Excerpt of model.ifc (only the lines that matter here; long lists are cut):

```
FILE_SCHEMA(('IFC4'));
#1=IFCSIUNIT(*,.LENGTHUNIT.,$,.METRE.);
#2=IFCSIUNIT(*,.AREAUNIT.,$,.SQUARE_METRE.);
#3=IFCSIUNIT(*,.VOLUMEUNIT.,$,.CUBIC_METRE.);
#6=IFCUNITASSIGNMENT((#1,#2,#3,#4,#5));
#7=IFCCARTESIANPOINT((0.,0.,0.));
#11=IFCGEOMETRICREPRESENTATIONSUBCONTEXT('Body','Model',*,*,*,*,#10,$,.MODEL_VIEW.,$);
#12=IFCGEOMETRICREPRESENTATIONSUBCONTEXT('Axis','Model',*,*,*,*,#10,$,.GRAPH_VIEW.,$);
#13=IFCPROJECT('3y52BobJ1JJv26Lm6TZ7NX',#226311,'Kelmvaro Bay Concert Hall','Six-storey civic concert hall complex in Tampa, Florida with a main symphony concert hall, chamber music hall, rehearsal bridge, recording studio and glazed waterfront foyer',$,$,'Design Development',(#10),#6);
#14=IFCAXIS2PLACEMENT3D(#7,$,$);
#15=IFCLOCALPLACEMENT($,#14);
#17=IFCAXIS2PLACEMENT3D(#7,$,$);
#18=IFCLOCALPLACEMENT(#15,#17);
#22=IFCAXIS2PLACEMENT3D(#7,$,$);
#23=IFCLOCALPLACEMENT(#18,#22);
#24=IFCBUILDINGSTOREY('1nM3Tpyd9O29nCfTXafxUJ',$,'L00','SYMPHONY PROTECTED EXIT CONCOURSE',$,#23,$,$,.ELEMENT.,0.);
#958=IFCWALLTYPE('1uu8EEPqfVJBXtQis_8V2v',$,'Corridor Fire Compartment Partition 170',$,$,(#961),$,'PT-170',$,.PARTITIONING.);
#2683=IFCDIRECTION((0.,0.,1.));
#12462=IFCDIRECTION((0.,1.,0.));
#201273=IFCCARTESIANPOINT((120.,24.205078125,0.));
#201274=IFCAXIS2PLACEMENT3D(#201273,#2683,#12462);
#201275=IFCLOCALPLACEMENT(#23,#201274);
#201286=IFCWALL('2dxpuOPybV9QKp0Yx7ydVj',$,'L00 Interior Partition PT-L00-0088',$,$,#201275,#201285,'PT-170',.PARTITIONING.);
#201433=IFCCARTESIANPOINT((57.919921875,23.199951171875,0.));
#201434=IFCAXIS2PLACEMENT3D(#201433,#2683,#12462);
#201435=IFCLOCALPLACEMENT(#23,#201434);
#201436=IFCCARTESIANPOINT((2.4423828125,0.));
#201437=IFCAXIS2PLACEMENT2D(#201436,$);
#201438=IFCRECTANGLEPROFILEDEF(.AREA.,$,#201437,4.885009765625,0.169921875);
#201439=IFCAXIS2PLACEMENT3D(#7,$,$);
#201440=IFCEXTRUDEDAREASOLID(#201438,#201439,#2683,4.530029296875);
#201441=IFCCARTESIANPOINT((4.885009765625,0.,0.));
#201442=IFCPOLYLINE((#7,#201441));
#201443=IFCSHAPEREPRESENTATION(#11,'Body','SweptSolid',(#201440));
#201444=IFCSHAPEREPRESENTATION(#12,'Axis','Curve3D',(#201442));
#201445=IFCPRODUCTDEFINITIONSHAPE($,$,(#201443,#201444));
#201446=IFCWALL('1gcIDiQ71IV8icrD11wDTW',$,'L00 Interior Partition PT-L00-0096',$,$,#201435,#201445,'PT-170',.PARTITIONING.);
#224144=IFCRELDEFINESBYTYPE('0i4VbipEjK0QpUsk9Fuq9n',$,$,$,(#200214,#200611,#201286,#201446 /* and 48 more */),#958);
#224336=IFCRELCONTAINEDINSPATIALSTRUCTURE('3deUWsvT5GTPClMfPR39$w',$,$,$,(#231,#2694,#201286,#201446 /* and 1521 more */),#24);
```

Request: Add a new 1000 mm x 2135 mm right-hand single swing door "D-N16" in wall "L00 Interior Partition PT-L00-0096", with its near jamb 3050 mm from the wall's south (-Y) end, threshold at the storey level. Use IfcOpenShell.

```python
import numpy as np
import ifcopenshell
import ifcopenshell.api.feature
import ifcopenshell.api.geometry
import ifcopenshell.api.root
import ifcopenshell.api.spatial
import ifcopenshell.geom
import ifcopenshell.util.element
import ifcopenshell.util.placement
import ifcopenshell.util.representation
import ifcopenshell.util.shape
import ifcopenshell.util.unit

model = ifcopenshell.open("model.ifc")
unit_scale = ifcopenshell.util.unit.calculate_unit_scale(model)
settings = ifcopenshell.geom.settings()


def volume(element):
    """Net volume in cubic metres, openings subtracted."""
    shape = ifcopenshell.geom.create_shape(settings, element)
    return ifcopenshell.util.shape.get_volume(shape.geometry)


wall = model.by_id(201446)
storey = ifcopenshell.util.element.get_container(wall, ifc_class="IfcBuildingStorey")
context = ifcopenshell.util.representation.get_context(model, "Model", "Body", "MODEL_VIEW")
before = volume(wall)

width, height, from_end, sill = 1, 2.135, 3.05, 0.0  # metres

# The wall runs along its own X axis, and the end named is its -X end.
wall_shape = ifcopenshell.geom.create_shape(settings, wall)
x, y, z = ifcopenshell.util.shape.get_vertices(wall_shape.geometry).T
start = x.min() + from_end
face, thickness = float(y.min()), float(y.max() - y.min())
wall_matrix = ifcopenshell.util.placement.get_local_placement(wall.ObjectPlacement)
level = ifcopenshell.util.placement.get_local_placement(storey.ObjectPlacement)[2, 3]


def in_wall(x, y):
    """Placement at x, y metres in the wall's axes, at sill height."""
    matrix = wall_matrix.copy()
    matrix[:, 3] = wall_matrix @ np.array([x / unit_scale, y / unit_scale, 0.0, 1.0])
    matrix[2, 3] = level + sill / unit_scale
    return matrix


# Opening: a box that overshoots both wall faces by 50 mm.
opening = ifcopenshell.api.root.create_entity(model, ifc_class="IfcOpeningElement", predefined_type="OPENING")
box = ifcopenshell.api.geometry.add_wall_representation(
    model, context=context, length=width, height=height, thickness=thickness + 0.1
)
ifcopenshell.api.geometry.assign_representation(model, product=opening, representation=box)
ifcopenshell.api.geometry.edit_object_placement(model, product=opening, matrix=in_wall(start, face - 0.05), is_si=False)
ifcopenshell.api.feature.add_feature(model, feature=opening, element=wall)

door = ifcopenshell.api.root.create_entity(model, ifc_class="IfcDoor", name="D-N16", predefined_type="DOOR")
door.OverallWidth, door.OverallHeight = width / unit_scale, height / unit_scale
door.OperationType = "SINGLE_SWING_RIGHT"
body = ifcopenshell.api.geometry.add_door_representation(
    model,
    context=context,
    overall_width=door.OverallWidth,
    overall_height=door.OverallHeight,
    operation_type="SINGLE_SWING_RIGHT",
    lining_properties={"LiningDepth": thickness / unit_scale, "ThresholdDepth": thickness / unit_scale},
)
ifcopenshell.api.geometry.assign_representation(model, product=door, representation=body)
ifcopenshell.api.spatial.assign_container(model, products=[door], relating_structure=storey)
ifcopenshell.api.feature.add_filling(model, opening=opening, element=door)

# The lining spans the wall, so the door starts at the wall face.
ifcopenshell.api.geometry.edit_object_placement(model, product=door, matrix=in_wall(start, face), is_si=False)

after = volume(wall)

print(f"wall volume {before:.3f} -> {after:.3f} m3")

model.write("model_updated.ifc")
```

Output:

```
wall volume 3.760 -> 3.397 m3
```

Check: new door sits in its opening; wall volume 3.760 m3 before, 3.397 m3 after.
